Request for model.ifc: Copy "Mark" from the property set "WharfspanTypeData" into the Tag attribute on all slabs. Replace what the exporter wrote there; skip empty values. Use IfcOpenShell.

First a look at what the model holds.

```python
import ifcopenshell
import ifcopenshell.util.element

model = ifcopenshell.open("model.ifc")
print(model.schema)
slabs = model.by_type("IfcSlab")
print(len(slabs), "slabs")
for e in slabs[:8]:
    source = ifcopenshell.util.element.get_pset(e, "WharfspanTypeData", "Mark")
    target = e.Tag
    print(e.id(), repr(source), repr(target), sep=" | ")
```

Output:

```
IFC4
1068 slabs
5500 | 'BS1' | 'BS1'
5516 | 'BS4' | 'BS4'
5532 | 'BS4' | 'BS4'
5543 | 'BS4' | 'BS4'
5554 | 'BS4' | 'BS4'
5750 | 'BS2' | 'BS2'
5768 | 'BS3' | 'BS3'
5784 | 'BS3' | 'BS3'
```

```python
import ifcopenshell
import ifcopenshell.util.element

model = ifcopenshell.open("model.ifc")

count = 0
for e in model.by_type("IfcSlab"):
    value = ifcopenshell.util.element.get_pset(e, "WharfspanTypeData", "Mark")
    current = e.Tag
    if not value or not value.strip() or current == value:
        continue
    e.Tag = value
    count += 1

print(count, "slabs updated")

model.write("model-out.ifc")
```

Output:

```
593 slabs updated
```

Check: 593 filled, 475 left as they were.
